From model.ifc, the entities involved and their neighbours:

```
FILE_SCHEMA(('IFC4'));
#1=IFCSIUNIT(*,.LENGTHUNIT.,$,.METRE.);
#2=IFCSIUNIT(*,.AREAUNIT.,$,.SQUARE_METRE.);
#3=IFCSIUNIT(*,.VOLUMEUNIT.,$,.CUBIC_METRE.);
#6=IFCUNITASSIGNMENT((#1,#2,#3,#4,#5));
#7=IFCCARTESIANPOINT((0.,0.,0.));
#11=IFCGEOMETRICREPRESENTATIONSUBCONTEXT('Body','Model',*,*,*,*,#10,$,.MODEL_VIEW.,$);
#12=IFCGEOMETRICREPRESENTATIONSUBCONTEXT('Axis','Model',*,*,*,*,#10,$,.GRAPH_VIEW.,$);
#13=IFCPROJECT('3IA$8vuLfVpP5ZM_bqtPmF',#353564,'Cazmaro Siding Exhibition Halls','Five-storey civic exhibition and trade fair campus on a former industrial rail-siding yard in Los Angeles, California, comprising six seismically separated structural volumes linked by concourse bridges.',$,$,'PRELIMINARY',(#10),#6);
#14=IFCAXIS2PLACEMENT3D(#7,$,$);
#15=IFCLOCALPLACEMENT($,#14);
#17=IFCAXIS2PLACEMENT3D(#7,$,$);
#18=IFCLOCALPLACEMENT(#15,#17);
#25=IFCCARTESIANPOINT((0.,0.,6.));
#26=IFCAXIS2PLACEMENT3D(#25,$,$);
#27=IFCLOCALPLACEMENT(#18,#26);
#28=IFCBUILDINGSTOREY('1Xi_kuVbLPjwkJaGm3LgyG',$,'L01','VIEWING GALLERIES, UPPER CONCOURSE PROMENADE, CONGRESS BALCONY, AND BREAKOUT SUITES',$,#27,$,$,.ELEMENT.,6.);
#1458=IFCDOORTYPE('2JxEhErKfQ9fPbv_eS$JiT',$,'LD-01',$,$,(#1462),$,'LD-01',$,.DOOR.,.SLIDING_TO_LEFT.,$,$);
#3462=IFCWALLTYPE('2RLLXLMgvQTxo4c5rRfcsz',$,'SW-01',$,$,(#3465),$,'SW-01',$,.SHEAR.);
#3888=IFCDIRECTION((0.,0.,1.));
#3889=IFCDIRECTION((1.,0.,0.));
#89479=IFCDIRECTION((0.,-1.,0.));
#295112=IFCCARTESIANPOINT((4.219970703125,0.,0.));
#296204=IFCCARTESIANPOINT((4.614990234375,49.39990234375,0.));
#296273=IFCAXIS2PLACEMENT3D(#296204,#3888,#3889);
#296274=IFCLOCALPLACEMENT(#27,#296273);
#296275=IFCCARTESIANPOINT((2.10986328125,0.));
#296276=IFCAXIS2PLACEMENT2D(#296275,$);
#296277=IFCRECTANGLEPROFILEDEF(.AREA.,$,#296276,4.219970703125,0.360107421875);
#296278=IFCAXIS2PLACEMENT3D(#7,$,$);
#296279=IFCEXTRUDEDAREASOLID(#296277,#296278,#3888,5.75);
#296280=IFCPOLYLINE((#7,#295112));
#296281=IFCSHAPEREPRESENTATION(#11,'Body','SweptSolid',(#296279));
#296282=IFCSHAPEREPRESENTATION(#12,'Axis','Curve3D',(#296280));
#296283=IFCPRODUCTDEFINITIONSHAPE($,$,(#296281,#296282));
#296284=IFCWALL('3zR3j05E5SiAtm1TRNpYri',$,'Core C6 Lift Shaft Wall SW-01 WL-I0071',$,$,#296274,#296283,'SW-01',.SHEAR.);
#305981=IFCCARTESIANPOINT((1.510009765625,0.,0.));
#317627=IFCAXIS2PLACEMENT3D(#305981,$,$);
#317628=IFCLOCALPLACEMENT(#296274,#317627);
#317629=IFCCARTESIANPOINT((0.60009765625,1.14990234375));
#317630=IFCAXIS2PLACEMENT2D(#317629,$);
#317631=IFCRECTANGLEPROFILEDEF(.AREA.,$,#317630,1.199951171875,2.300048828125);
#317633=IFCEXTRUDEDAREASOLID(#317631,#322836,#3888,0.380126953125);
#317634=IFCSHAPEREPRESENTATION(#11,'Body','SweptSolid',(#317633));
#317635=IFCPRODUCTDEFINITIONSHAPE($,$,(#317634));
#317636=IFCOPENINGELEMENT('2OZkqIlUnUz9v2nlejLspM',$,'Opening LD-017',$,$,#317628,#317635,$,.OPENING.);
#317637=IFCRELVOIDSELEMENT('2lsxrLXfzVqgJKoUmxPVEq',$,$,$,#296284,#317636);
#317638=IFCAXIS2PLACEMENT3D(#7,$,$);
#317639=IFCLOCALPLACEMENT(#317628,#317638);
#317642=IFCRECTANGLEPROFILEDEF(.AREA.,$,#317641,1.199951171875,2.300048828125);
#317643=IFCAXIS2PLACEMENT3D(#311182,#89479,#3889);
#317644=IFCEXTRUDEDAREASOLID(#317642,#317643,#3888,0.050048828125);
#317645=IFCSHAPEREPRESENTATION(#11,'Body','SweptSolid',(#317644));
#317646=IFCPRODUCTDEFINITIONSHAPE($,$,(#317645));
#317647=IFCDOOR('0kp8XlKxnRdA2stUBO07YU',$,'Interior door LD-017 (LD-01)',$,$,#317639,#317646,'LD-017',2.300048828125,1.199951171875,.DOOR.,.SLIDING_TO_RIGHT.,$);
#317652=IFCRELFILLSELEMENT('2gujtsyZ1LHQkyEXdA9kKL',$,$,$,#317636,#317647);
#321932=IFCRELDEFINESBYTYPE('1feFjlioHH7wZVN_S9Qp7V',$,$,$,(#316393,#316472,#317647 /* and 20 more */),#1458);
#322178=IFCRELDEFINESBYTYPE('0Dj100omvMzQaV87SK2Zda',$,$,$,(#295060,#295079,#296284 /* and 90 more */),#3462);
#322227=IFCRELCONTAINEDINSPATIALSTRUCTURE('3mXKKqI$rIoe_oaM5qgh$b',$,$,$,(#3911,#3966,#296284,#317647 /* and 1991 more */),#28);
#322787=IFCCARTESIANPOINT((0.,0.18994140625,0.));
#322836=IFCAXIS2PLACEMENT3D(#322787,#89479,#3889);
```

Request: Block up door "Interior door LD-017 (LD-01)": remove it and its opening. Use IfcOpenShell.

```python
import ifcopenshell
import ifcopenshell.api.feature
import ifcopenshell.api.root
import ifcopenshell.geom
import ifcopenshell.util.shape

model = ifcopenshell.open("model.ifc")
settings = ifcopenshell.geom.settings()


def volume(element):
    """Net volume in cubic metres, openings subtracted."""
    shape = ifcopenshell.geom.create_shape(settings, element)
    return ifcopenshell.util.shape.get_volume(shape.geometry)


door = model.by_guid("0kp8XlKxnRdA2stUBO07YU")
opening = door.FillsVoids[0].RelatingOpeningElement
wall = opening.VoidsElements[0].RelatingBuildingElement
before = volume(wall)

ifcopenshell.api.root.remove_product(model, product=door)
ifcopenshell.api.feature.remove_feature(model, feature=opening)

after = volume(wall)

print(f"wall volume {before:.3f} -> {after:.3f} m3")

model.write("model_updated.ifc")
```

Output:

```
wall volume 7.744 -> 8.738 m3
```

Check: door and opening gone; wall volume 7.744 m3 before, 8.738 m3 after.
